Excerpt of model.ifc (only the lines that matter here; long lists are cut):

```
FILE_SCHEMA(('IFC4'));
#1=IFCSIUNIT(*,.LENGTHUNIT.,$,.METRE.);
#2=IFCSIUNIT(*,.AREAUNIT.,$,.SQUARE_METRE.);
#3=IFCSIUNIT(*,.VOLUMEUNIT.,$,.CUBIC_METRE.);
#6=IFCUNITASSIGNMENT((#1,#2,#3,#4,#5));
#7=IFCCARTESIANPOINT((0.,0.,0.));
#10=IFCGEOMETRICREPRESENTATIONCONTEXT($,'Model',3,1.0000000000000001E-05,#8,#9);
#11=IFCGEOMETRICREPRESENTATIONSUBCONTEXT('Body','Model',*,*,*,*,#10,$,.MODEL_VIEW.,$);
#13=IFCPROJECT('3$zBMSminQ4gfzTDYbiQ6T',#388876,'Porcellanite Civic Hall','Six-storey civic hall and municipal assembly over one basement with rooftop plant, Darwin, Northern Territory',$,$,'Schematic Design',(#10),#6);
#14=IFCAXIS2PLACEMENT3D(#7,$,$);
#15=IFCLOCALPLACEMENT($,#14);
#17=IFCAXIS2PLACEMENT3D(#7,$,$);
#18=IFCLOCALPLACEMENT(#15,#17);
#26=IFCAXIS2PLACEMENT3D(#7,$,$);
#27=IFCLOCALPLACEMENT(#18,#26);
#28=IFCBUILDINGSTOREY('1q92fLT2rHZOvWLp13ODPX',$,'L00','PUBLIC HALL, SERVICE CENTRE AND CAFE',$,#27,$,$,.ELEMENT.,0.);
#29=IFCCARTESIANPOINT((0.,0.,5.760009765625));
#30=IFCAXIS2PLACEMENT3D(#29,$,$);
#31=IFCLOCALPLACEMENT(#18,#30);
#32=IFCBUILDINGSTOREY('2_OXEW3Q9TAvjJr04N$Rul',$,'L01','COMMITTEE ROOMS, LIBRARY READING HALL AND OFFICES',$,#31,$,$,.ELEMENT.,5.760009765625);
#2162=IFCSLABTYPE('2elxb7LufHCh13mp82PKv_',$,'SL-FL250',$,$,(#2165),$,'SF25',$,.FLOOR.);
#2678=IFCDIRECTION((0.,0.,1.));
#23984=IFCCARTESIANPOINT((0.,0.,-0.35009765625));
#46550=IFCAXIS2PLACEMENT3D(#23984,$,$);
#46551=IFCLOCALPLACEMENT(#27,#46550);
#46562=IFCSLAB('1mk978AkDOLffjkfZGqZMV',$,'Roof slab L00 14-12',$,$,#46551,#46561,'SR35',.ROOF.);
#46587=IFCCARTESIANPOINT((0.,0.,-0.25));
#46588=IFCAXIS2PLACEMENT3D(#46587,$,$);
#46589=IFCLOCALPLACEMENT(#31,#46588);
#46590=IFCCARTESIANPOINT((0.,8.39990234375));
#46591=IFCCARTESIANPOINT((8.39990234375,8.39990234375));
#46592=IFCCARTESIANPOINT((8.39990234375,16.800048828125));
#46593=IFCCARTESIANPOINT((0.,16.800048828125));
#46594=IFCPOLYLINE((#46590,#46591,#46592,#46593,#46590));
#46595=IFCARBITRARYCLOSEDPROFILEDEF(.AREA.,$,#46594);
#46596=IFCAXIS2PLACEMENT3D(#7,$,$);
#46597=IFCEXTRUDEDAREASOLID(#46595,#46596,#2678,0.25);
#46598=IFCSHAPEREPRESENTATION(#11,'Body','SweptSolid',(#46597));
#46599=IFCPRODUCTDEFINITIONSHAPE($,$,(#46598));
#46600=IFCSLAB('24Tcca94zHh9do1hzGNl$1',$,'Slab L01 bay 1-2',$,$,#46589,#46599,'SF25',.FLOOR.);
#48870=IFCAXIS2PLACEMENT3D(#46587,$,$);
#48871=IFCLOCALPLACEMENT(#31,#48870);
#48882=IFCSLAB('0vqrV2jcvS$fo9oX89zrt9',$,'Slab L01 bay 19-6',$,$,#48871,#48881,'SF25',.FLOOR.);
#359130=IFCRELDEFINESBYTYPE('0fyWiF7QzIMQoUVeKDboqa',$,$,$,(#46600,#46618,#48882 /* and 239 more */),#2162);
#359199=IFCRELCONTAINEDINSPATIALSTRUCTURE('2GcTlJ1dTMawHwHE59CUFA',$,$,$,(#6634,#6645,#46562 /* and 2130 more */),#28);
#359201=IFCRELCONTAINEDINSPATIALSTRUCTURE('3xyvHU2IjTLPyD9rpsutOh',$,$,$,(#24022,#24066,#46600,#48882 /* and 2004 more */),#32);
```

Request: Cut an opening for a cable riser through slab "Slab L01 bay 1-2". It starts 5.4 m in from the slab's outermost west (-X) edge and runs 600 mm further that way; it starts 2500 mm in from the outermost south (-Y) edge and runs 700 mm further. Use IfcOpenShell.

```python
import numpy as np
import ifcopenshell
import ifcopenshell.api.feature
import ifcopenshell.api.geometry
import ifcopenshell.api.root
import ifcopenshell.geom
import ifcopenshell.util.placement
import ifcopenshell.util.representation
import ifcopenshell.util.shape
import ifcopenshell.util.unit

model = ifcopenshell.open("model.ifc")
unit_scale = ifcopenshell.util.unit.calculate_unit_scale(model)
settings = ifcopenshell.geom.settings()


def volume(element):
    """Net volume in cubic metres, openings subtracted."""
    shape = ifcopenshell.geom.create_shape(settings, element)
    return ifcopenshell.util.shape.get_volume(shape.geometry)


slab = model.by_id(46600)
before = volume(slab)

# Extent in the slab's own axes, in metres. The edges named are its -X and -Y sides.
slab_shape = ifcopenshell.geom.create_shape(settings, slab)
vertices = ifcopenshell.util.shape.get_vertices(slab_shape.geometry)
x_min, y_min, bottom = vertices.min(axis=0)
top = vertices[:, 2].max()

opening = ifcopenshell.api.root.create_entity(model, ifc_class="IfcOpeningElement", name="Cable riser opening", predefined_type="OPENING")
context = ifcopenshell.util.representation.get_context(model, "Model", "Body", "MODEL_VIEW")
width, depth = 0.6, 0.7
outline = [(0.0, 0.0), (width, 0.0), (width, depth), (0.0, depth), (0.0, 0.0)]
# Overshoot both faces by 50 mm so the cut is clean.
shape = ifcopenshell.api.geometry.add_slab_representation(
    model, context=context, depth=top - bottom + 0.1, polyline=outline
)
ifcopenshell.api.geometry.assign_representation(model, product=opening, representation=shape)

matrix = ifcopenshell.util.placement.get_local_placement(slab.ObjectPlacement)
matrix[:, 3] = matrix @ np.append(np.array([x_min + 5.4, y_min + 2.5, bottom - 0.05]) / unit_scale, 1.0)
ifcopenshell.api.geometry.edit_object_placement(model, product=opening, matrix=matrix, is_si=False)
ifcopenshell.api.feature.add_feature(model, feature=opening, element=slab)

after = volume(slab)

print(f"slab volume {before:.3f} -> {after:.3f} m3")

model.write("model_edited.ifc")
```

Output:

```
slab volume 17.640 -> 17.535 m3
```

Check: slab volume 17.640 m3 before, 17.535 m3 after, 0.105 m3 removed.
